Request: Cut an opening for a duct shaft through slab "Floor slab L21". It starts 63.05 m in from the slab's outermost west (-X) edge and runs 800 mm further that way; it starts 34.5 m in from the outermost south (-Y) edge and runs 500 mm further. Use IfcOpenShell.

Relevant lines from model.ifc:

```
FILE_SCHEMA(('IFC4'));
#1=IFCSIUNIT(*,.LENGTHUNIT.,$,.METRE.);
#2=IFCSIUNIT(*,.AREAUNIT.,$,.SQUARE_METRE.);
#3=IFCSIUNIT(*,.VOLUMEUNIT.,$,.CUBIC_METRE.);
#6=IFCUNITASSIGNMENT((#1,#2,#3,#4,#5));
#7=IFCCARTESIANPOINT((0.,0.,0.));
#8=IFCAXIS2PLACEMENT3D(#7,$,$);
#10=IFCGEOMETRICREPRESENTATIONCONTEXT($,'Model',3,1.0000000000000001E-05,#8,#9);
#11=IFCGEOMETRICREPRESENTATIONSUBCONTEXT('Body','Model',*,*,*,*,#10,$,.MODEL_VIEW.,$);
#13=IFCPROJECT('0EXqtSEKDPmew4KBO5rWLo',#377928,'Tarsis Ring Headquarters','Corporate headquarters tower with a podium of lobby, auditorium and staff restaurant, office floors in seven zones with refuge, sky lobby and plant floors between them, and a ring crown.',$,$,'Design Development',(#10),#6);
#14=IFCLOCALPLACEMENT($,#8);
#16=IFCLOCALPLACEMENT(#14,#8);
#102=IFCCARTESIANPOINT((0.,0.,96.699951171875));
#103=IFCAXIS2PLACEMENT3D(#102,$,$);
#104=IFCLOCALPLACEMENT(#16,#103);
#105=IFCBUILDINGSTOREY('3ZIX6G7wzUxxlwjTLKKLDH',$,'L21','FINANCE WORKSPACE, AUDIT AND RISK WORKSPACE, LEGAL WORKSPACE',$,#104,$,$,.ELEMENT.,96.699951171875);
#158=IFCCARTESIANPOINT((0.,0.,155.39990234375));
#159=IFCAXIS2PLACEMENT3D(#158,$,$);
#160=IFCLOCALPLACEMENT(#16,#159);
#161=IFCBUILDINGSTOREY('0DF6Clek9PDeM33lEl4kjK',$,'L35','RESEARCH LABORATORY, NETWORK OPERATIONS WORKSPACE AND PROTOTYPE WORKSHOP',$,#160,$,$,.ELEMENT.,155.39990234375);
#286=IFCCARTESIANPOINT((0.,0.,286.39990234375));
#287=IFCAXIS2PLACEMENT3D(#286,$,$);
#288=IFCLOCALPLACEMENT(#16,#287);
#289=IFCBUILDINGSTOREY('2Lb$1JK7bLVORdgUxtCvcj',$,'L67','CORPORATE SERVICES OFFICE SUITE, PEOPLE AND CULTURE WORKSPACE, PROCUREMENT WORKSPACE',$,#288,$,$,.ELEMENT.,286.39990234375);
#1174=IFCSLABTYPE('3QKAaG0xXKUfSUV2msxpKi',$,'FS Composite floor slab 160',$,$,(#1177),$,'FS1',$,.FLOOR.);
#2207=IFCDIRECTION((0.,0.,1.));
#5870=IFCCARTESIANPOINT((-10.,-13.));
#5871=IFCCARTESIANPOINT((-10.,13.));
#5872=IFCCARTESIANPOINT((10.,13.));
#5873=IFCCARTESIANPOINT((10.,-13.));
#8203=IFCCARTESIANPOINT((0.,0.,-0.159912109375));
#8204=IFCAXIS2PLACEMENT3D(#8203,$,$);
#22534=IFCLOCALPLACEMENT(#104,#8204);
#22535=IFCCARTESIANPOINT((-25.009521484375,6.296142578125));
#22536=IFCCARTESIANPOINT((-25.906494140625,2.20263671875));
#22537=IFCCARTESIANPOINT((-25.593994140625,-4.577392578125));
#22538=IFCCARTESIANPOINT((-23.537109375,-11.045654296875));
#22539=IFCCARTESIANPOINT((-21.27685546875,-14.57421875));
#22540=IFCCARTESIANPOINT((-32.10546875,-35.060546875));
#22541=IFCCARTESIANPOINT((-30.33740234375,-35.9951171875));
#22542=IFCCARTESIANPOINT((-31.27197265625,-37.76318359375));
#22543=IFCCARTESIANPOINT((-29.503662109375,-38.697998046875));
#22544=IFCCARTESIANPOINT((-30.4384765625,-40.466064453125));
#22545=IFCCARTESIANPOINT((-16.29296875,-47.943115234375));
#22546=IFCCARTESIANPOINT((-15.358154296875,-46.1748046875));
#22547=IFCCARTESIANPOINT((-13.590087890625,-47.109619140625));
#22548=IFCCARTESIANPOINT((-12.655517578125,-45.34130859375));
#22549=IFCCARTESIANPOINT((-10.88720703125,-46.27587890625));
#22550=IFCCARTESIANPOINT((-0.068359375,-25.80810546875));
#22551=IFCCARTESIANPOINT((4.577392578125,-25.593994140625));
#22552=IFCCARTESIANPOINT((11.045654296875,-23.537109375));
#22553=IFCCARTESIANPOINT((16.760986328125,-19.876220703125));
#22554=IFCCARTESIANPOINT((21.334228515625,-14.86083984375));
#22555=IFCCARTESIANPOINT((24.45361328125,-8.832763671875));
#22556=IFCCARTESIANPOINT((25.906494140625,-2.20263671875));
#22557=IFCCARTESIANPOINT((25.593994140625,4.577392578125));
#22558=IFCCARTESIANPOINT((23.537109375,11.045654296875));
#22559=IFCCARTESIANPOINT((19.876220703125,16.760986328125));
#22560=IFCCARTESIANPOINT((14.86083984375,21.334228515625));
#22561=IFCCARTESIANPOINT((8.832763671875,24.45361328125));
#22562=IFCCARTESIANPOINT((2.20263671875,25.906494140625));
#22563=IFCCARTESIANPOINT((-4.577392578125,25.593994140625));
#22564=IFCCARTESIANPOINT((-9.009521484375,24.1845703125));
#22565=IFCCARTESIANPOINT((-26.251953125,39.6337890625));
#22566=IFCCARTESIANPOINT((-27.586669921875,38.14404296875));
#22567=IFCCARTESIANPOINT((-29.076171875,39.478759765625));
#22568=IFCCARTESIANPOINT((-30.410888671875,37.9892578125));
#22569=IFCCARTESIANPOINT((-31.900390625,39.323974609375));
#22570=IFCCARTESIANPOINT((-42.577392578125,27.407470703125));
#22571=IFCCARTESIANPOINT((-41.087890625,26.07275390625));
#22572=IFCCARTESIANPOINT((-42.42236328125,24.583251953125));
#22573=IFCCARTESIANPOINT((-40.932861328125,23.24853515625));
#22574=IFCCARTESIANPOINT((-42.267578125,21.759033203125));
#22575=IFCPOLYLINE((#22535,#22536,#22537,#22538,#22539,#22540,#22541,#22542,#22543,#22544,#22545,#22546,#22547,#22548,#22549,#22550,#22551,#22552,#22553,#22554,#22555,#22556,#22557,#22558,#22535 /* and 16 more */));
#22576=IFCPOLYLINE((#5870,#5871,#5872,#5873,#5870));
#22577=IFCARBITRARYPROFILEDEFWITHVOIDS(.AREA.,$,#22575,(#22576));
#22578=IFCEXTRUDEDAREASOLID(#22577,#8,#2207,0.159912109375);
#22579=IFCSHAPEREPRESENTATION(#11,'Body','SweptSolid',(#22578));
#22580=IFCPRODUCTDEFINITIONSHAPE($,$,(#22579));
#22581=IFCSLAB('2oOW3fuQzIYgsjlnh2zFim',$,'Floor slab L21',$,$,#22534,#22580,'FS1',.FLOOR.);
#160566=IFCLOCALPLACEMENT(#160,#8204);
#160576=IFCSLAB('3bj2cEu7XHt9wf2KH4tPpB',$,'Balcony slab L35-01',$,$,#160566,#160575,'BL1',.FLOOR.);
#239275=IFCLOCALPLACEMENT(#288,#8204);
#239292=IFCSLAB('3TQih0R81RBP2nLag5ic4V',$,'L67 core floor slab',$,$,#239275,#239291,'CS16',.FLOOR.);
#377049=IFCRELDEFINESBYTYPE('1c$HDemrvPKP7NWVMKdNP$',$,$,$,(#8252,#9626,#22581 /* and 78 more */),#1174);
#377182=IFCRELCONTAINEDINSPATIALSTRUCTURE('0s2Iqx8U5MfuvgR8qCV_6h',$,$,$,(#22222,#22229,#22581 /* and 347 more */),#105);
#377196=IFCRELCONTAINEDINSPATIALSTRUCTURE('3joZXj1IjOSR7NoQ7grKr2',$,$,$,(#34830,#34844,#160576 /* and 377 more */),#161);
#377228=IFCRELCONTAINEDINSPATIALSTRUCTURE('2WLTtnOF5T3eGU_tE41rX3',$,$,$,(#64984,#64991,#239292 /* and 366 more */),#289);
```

```python
import numpy as np
import ifcopenshell
import ifcopenshell.api.feature
import ifcopenshell.api.geometry
import ifcopenshell.api.root
import ifcopenshell.geom
import ifcopenshell.util.placement
import ifcopenshell.util.representation
import ifcopenshell.util.shape
import ifcopenshell.util.unit

model = ifcopenshell.open("model.ifc")
unit_scale = ifcopenshell.util.unit.calculate_unit_scale(model)
settings = ifcopenshell.geom.settings()


def volume(element):
    """Net volume in cubic metres, openings subtracted."""
    shape = ifcopenshell.geom.create_shape(settings, element)
    return ifcopenshell.util.shape.get_volume(shape.geometry)


slab = model.by_guid("2oOW3fuQzIYgsjlnh2zFim")
before = volume(slab)

# Extent in the slab's own axes, in metres. The edges named are its -X and -Y sides.
slab_shape = ifcopenshell.geom.create_shape(settings, slab)
vertices = ifcopenshell.util.shape.get_vertices(slab_shape.geometry)
x_min, y_min, bottom = vertices.min(axis=0)
top = vertices[:, 2].max()

opening = ifcopenshell.api.root.create_entity(model, ifc_class="IfcOpeningElement", name="Duct shaft opening", predefined_type="OPENING")
context = ifcopenshell.util.representation.get_context(model, "Model", "Body", "MODEL_VIEW")
width, depth = 0.8, 0.5
outline = [(0.0, 0.0), (width, 0.0), (width, depth), (0.0, depth), (0.0, 0.0)]
# Overshoot both faces by 50 mm so the cut is clean.
shape = ifcopenshell.api.geometry.add_slab_representation(
    model, context=context, depth=top - bottom + 0.1, polyline=outline
)
ifcopenshell.api.geometry.assign_representation(model, product=opening, representation=shape)

matrix = ifcopenshell.util.placement.get_local_placement(slab.ObjectPlacement)
matrix[:, 3] = matrix @ np.append(np.array([x_min + 63.05, y_min + 34.5, bottom - 0.05]) / unit_scale, 1.0)
ifcopenshell.api.geometry.edit_object_placement(model, product=opening, matrix=matrix, is_si=False)
ifcopenshell.api.feature.add_feature(model, feature=opening, element=slab)

after = volume(slab)

print(f"slab volume {before:.3f} -> {after:.3f} m3")

model.write("model-out.ifc")
```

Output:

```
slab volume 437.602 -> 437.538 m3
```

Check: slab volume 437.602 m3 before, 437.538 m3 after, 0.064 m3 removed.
